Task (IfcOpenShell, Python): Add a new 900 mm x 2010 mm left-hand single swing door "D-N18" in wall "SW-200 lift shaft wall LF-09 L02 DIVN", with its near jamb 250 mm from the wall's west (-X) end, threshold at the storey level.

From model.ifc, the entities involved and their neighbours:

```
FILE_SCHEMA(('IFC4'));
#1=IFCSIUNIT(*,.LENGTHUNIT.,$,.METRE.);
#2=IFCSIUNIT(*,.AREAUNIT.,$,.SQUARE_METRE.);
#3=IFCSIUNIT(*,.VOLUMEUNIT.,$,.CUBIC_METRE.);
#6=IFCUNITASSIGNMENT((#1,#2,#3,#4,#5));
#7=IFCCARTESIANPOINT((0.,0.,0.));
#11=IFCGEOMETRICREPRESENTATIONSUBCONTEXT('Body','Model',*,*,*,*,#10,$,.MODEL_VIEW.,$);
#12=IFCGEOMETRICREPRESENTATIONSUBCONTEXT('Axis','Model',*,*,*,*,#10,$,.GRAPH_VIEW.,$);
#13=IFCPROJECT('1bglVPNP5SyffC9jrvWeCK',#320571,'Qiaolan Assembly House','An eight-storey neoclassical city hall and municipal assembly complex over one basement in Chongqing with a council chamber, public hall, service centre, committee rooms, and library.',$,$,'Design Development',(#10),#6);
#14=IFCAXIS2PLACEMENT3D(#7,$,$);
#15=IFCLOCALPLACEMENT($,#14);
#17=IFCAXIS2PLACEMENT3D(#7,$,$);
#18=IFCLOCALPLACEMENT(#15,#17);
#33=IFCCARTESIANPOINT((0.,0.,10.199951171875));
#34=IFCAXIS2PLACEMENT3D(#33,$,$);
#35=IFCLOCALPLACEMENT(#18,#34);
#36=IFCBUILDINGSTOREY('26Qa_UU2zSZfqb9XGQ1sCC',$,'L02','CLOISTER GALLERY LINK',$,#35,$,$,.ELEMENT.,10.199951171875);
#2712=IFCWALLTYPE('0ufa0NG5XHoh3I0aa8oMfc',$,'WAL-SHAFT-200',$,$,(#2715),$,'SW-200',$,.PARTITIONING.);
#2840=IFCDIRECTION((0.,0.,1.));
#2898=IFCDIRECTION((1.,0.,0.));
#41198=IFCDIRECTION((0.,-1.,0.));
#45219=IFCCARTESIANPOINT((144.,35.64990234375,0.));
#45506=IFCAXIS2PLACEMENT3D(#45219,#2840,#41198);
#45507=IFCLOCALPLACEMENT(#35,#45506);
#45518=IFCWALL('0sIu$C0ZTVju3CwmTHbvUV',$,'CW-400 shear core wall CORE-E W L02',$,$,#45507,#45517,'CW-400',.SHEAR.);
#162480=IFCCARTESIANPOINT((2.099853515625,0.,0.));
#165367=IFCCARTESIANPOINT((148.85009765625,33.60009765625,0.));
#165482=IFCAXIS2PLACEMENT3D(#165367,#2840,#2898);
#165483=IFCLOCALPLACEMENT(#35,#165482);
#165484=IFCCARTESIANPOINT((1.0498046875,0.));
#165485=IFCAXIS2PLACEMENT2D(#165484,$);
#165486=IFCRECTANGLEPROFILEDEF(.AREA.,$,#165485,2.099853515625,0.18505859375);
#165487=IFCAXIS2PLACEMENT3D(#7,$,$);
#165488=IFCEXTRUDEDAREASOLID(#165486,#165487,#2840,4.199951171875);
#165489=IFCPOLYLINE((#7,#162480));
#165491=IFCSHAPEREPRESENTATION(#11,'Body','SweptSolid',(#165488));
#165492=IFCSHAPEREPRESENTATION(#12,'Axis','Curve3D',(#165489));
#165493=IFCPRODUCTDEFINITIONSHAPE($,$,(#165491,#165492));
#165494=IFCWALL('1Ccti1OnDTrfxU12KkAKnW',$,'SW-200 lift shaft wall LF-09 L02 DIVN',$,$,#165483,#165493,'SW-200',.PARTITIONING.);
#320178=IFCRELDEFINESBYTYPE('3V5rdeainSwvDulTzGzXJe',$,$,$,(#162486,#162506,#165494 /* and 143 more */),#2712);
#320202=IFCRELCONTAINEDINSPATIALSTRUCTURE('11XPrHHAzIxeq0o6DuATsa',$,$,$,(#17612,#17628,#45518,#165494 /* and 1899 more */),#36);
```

```python
import numpy as np
import ifcopenshell
import ifcopenshell.api.feature
import ifcopenshell.api.geometry
import ifcopenshell.api.root
import ifcopenshell.api.spatial
import ifcopenshell.geom
import ifcopenshell.util.element
import ifcopenshell.util.placement
import ifcopenshell.util.representation
import ifcopenshell.util.shape
import ifcopenshell.util.unit

model = ifcopenshell.open("model.ifc")
unit_scale = ifcopenshell.util.unit.calculate_unit_scale(model)
settings = ifcopenshell.geom.settings()


def volume(element):
    """Net volume in cubic metres, openings subtracted."""
    shape = ifcopenshell.geom.create_shape(settings, element)
    return ifcopenshell.util.shape.get_volume(shape.geometry)


wall = model.by_guid("1Ccti1OnDTrfxU12KkAKnW")
storey = ifcopenshell.util.element.get_container(wall, ifc_class="IfcBuildingStorey")
context = ifcopenshell.util.representation.get_context(model, "Model", "Body", "MODEL_VIEW")
before = volume(wall)

width, height, from_end, sill = 0.9, 2.01, 0.25, 0.0  # metres

# The wall runs along its own X axis, and the end named is its -X end.
wall_shape = ifcopenshell.geom.create_shape(settings, wall)
x, y, z = ifcopenshell.util.shape.get_vertices(wall_shape.geometry).T
start = x.min() + from_end
face, thickness = float(y.min()), float(y.max() - y.min())
wall_matrix = ifcopenshell.util.placement.get_local_placement(wall.ObjectPlacement)
level = ifcopenshell.util.placement.get_local_placement(storey.ObjectPlacement)[2, 3]


def in_wall(x, y):
    """Placement at x, y metres in the wall's axes, at sill height."""
    matrix = wall_matrix.copy()
    matrix[:, 3] = wall_matrix @ np.array([x / unit_scale, y / unit_scale, 0.0, 1.0])
    matrix[2, 3] = level + sill / unit_scale
    return matrix


# Opening: a box that overshoots both wall faces by 50 mm.
opening = ifcopenshell.api.root.create_entity(model, ifc_class="IfcOpeningElement", predefined_type="OPENING")
box = ifcopenshell.api.geometry.add_wall_representation(
    model, context=context, length=width, height=height, thickness=thickness + 0.1
)
ifcopenshell.api.geometry.assign_representation(model, product=opening, representation=box)
ifcopenshell.api.geometry.edit_object_placement(model, product=opening, matrix=in_wall(start, face - 0.05), is_si=False)
ifcopenshell.api.feature.add_feature(model, feature=opening, element=wall)

door = ifcopenshell.api.root.create_entity(model, ifc_class="IfcDoor", name="D-N18", predefined_type="DOOR")
door.OverallWidth, door.OverallHeight = width / unit_scale, height / unit_scale
door.OperationType = "SINGLE_SWING_LEFT"
body = ifcopenshell.api.geometry.add_door_representation(
    model,
    context=context,
    overall_width=door.OverallWidth,
    overall_height=door.OverallHeight,
    operation_type="SINGLE_SWING_LEFT",
    lining_properties={"LiningDepth": thickness / unit_scale, "ThresholdDepth": thickness / unit_scale},
)
ifcopenshell.api.geometry.assign_representation(model, product=door, representation=body)
ifcopenshell.api.spatial.assign_container(model, products=[door], relating_structure=storey)
ifcopenshell.api.feature.add_filling(model, opening=opening, element=door)

# The lining spans the wall, so the door starts at the wall face.
ifcopenshell.api.geometry.edit_object_placement(model, product=door, matrix=in_wall(start, face), is_si=False)

after = volume(wall)

print(f"wall volume {before:.3f} -> {after:.3f} m3")

model.write("model_updated.ifc")
```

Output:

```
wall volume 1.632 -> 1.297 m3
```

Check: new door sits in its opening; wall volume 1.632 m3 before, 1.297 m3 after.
